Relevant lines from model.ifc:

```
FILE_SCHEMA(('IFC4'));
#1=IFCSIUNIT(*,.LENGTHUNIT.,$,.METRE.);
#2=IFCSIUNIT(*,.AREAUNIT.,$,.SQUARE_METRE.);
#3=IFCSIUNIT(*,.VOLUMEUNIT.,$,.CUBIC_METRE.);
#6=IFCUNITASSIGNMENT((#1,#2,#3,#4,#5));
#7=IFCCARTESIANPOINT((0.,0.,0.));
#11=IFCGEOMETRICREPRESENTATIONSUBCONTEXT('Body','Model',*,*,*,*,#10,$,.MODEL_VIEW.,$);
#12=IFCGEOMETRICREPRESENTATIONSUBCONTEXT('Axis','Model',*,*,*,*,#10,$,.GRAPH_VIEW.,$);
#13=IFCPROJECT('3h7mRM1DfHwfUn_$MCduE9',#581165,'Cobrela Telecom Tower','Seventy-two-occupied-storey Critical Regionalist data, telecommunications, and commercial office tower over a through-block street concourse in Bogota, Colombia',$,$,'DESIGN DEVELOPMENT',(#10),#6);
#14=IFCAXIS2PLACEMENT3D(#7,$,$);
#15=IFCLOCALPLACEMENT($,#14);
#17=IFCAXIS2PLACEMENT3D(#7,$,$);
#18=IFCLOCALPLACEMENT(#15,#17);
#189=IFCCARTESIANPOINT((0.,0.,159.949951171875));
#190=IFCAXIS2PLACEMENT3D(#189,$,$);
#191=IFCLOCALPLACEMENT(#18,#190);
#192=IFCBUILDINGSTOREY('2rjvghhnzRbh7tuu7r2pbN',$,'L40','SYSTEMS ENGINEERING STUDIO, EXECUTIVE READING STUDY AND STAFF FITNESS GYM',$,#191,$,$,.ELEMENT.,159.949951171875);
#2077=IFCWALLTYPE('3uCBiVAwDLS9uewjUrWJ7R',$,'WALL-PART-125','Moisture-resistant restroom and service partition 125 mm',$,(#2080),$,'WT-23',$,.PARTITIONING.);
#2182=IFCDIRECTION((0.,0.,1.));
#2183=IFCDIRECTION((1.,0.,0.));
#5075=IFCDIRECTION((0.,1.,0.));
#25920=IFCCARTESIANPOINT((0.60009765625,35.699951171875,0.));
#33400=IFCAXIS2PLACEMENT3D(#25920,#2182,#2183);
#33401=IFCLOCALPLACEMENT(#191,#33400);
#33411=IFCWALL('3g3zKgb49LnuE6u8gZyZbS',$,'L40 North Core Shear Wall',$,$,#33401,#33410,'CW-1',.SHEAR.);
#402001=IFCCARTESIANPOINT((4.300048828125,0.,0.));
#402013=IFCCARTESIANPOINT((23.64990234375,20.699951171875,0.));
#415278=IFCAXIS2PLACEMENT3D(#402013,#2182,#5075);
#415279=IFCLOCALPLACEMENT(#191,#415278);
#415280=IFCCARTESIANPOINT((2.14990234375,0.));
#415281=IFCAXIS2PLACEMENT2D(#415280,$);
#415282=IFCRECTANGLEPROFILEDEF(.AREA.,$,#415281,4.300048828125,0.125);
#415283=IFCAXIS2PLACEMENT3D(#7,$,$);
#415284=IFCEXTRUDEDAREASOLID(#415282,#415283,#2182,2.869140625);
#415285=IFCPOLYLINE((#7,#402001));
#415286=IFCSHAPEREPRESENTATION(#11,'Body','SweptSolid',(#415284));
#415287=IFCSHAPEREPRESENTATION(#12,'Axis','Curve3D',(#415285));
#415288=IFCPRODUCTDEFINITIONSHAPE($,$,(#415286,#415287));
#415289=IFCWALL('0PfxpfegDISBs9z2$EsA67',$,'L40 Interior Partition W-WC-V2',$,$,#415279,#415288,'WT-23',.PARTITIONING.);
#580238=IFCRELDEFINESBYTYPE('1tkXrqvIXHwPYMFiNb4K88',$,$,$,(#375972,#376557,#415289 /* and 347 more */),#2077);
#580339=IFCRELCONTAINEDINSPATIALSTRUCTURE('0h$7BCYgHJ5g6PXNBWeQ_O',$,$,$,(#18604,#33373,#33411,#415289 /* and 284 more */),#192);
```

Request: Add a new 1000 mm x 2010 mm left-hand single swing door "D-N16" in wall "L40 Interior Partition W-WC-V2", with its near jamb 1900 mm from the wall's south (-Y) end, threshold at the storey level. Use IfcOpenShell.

```python
import numpy as np
import ifcopenshell
import ifcopenshell.api.feature
import ifcopenshell.api.geometry
import ifcopenshell.api.root
import ifcopenshell.api.spatial
import ifcopenshell.geom
import ifcopenshell.util.element
import ifcopenshell.util.placement
import ifcopenshell.util.representation
import ifcopenshell.util.shape
import ifcopenshell.util.unit

model = ifcopenshell.open("model.ifc")
unit_scale = ifcopenshell.util.unit.calculate_unit_scale(model)
settings = ifcopenshell.geom.settings()


def volume(element):
    """Net volume in cubic metres, openings subtracted."""
    shape = ifcopenshell.geom.create_shape(settings, element)
    return ifcopenshell.util.shape.get_volume(shape.geometry)


wall = model.by_guid("0PfxpfegDISBs9z2$EsA67")
storey = ifcopenshell.util.element.get_container(wall, ifc_class="IfcBuildingStorey")
context = ifcopenshell.util.representation.get_context(model, "Model", "Body", "MODEL_VIEW")
before = volume(wall)

width, height, from_end, sill = 1, 2.01, 1.9, 0.0  # metres

# The wall runs along its own X axis, and the end named is its -X end.
wall_shape = ifcopenshell.geom.create_shape(settings, wall)
x, y, z = ifcopenshell.util.shape.get_vertices(wall_shape.geometry).T
start = x.min() + from_end
face, thickness = float(y.min()), float(y.max() - y.min())
wall_matrix = ifcopenshell.util.placement.get_local_placement(wall.ObjectPlacement)
level = ifcopenshell.util.placement.get_local_placement(storey.ObjectPlacement)[2, 3]


def in_wall(x, y):
    """Placement at x, y metres in the wall's axes, at sill height."""
    matrix = wall_matrix.copy()
    matrix[:, 3] = wall_matrix @ np.array([x / unit_scale, y / unit_scale, 0.0, 1.0])
    matrix[2, 3] = level + sill / unit_scale
    return matrix


# Opening: a box that overshoots both wall faces by 50 mm.
opening = ifcopenshell.api.root.create_entity(model, ifc_class="IfcOpeningElement", predefined_type="OPENING")
box = ifcopenshell.api.geometry.add_wall_representation(
    model, context=context, length=width, height=height, thickness=thickness + 0.1
)
ifcopenshell.api.geometry.assign_representation(model, product=opening, representation=box)
ifcopenshell.api.geometry.edit_object_placement(model, product=opening, matrix=in_wall(start, face - 0.05), is_si=False)
ifcopenshell.api.feature.add_feature(model, feature=opening, element=wall)

door = ifcopenshell.api.root.create_entity(model, ifc_class="IfcDoor", name="D-N16", predefined_type="DOOR")
door.OverallWidth, door.OverallHeight = width / unit_scale, height / unit_scale
door.OperationType = "SINGLE_SWING_LEFT"
body = ifcopenshell.api.geometry.add_door_representation(
    model,
    context=context,
    overall_width=door.OverallWidth,
    overall_height=door.OverallHeight,
    operation_type="SINGLE_SWING_LEFT",
    lining_properties={"LiningDepth": thickness / unit_scale, "ThresholdDepth": thickness / unit_scale},
)
ifcopenshell.api.geometry.assign_representation(model, product=door, representation=body)
ifcopenshell.api.spatial.assign_container(model, products=[door], relating_structure=storey)
ifcopenshell.api.feature.add_filling(model, opening=opening, element=door)

# The lining spans the wall, so the door starts at the wall face.
ifcopenshell.api.geometry.edit_object_placement(model, product=door, matrix=in_wall(start, face), is_si=False)

after = volume(wall)

print(f"wall volume {before:.3f} -> {after:.3f} m3")

model.write("model_rev.ifc")
```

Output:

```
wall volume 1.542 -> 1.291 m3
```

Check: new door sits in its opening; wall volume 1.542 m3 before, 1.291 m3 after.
